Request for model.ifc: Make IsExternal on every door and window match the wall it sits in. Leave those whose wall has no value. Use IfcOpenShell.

First a look at what the model holds.

```python
import ifcopenshell
import ifcopenshell.util.element

model = ifcopenshell.open("model.ifc")
print(model.schema)
seen = {}
for e in model.by_type("IfcDoor") + model.by_type("IfcWindow"):
    if not e.FillsVoids:
        continue
    host = e.FillsVoids[0].RelatingOpeningElement.VoidsElements[0].RelatingBuildingElement
    own = ifcopenshell.util.element.get_pset(e, f"Pset_{e.is_a()[3:].removesuffix('StandardCase')}Common", "IsExternal")
    wall = ifcopenshell.util.element.get_pset(host, "Pset_WallCommon", "IsExternal")
    seen[e.is_a(), own, wall] = seen.get((e.is_a(), own, wall), 0) + 1
for (cls, own, wall), count in sorted(seen.items(), key=str):
    print(count, cls, "IsExternal:", own, "| host wall:", wall)
```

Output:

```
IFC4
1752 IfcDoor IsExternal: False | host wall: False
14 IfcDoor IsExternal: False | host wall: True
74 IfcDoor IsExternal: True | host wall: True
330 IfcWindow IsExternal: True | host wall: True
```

```python
import ifcopenshell
import ifcopenshell.api.pset
import ifcopenshell.util.element

model = ifcopenshell.open("model.ifc")

count = 0
for ifc_class, pset_name in (("IfcDoor", "Pset_DoorCommon"), ("IfcWindow", "Pset_WindowCommon")):
    for e in model.by_type(ifc_class):
        if not e.FillsVoids:
            continue
        host = e.FillsVoids[0].RelatingOpeningElement.VoidsElements[0].RelatingBuildingElement
        external = ifcopenshell.util.element.get_pset(host, "Pset_WallCommon", "IsExternal")
        if external is None or ifcopenshell.util.element.get_pset(e, pset_name, "IsExternal") == external:
            continue
        pset = ifcopenshell.api.pset.add_pset(model, product=e, name=pset_name)
        ifcopenshell.api.pset.edit_pset(model, pset=pset, properties={"IsExternal": external})
        count += 1

print(count, "updated")

model.write("model_rev.ifc")
```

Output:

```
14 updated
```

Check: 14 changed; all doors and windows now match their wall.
